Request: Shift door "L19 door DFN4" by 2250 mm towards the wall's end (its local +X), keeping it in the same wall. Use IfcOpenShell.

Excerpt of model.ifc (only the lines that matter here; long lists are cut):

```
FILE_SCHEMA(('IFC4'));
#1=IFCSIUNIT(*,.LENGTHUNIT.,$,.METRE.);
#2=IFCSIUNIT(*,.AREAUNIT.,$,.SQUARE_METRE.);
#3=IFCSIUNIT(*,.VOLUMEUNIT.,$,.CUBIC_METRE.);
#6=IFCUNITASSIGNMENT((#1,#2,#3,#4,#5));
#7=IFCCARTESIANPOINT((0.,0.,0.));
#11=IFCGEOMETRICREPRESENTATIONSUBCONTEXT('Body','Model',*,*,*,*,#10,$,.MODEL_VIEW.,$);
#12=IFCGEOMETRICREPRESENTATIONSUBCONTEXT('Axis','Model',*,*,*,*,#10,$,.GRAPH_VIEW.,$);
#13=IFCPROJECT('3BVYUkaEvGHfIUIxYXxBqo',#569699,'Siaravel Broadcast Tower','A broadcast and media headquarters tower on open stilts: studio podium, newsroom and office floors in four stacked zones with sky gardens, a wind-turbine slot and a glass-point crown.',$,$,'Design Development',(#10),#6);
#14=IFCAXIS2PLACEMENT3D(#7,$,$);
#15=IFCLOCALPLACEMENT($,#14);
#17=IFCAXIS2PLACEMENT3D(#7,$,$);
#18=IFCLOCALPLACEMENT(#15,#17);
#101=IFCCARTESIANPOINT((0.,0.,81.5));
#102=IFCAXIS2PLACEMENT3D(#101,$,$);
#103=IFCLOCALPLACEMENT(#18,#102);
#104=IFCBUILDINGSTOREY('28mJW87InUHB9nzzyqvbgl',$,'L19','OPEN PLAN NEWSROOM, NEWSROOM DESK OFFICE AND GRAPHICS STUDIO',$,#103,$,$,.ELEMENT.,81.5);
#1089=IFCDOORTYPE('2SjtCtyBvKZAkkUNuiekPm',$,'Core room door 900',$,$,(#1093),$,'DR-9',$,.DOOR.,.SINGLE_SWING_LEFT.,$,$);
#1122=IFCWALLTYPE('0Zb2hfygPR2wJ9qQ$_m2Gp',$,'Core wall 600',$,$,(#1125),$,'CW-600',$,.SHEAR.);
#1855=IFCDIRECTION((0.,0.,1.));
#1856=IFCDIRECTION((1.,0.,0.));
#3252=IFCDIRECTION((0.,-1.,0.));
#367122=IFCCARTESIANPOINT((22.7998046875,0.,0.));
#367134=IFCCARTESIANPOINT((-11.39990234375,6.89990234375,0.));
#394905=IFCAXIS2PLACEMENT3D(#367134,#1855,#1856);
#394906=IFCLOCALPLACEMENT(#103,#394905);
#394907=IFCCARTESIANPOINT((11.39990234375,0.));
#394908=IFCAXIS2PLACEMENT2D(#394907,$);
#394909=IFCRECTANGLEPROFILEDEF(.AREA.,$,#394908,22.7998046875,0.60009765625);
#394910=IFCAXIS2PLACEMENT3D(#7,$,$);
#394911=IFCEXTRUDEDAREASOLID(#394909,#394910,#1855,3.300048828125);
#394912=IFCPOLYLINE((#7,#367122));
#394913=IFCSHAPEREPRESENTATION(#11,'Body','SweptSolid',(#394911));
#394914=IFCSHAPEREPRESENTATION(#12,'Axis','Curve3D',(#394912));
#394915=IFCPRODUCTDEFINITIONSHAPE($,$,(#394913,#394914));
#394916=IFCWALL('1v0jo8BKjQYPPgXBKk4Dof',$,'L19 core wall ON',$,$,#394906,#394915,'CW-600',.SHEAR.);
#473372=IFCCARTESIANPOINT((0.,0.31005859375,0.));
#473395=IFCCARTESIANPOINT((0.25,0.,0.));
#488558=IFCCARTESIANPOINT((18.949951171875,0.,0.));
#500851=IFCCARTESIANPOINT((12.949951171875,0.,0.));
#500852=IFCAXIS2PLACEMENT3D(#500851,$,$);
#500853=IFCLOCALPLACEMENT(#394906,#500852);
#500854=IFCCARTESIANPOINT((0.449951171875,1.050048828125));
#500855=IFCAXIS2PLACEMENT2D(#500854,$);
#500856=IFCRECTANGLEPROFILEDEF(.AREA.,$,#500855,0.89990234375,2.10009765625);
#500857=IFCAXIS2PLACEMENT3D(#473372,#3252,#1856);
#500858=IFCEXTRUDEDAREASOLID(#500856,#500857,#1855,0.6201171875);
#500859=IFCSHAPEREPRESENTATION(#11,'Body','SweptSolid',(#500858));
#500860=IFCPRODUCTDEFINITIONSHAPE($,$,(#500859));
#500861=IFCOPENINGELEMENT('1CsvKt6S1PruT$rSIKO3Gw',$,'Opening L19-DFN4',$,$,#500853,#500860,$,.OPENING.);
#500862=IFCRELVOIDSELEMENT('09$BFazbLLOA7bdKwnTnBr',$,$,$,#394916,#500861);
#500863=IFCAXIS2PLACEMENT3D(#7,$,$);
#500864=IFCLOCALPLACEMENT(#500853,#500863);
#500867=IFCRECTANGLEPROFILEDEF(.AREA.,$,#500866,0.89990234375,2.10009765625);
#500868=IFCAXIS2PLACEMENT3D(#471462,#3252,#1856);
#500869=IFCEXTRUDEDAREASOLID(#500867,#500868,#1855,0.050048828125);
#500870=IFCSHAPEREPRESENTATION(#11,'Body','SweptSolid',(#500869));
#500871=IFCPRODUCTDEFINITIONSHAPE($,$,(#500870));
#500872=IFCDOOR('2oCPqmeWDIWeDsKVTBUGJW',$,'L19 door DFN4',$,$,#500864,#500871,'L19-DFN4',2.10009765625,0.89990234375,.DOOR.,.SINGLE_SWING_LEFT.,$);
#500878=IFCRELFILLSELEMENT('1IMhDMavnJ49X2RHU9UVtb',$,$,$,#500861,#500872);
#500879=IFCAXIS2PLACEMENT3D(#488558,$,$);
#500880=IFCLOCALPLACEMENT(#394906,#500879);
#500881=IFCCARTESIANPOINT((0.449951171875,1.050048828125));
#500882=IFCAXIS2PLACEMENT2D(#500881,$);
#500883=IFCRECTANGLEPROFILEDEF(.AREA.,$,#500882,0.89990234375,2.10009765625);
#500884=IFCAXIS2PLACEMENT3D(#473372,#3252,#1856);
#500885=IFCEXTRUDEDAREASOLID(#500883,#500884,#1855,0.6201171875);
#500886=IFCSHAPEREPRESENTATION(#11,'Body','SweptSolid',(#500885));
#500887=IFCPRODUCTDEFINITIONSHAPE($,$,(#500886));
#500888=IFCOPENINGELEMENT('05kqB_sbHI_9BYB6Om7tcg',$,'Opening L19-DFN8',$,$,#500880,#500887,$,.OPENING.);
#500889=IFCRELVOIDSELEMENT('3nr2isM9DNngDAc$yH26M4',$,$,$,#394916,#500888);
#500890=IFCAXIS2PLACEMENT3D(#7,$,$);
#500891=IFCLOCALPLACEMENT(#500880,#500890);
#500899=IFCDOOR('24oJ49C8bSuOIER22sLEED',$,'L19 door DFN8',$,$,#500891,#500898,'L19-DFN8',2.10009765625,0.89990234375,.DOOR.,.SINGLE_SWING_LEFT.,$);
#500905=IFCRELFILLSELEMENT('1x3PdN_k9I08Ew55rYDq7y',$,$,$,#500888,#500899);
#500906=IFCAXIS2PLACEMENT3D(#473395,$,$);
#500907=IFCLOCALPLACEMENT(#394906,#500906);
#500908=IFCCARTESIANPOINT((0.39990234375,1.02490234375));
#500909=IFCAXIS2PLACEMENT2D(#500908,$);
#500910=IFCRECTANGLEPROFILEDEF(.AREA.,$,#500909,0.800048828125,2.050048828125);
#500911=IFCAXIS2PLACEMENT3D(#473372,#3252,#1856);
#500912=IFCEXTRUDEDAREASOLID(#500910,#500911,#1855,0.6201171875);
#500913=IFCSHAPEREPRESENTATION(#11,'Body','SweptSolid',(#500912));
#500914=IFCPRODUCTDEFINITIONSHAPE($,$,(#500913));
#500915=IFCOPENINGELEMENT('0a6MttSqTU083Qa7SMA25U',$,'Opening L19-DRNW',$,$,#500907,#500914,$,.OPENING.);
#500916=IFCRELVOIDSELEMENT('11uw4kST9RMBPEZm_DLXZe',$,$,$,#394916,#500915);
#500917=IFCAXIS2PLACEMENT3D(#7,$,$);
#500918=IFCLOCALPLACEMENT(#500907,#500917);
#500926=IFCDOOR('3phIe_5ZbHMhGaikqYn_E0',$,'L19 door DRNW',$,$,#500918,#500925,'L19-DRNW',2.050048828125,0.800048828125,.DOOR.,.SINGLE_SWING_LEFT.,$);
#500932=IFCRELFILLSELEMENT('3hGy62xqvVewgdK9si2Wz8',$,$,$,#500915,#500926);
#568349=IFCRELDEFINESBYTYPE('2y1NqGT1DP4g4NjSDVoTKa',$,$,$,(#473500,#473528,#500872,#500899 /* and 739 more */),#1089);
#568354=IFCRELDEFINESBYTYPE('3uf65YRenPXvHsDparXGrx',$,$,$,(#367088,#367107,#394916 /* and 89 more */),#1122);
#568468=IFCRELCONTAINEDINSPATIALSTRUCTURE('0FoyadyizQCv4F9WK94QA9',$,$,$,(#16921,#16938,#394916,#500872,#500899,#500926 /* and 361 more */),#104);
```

```python
import ifcopenshell
import ifcopenshell.api.geometry
import ifcopenshell.util.placement
import ifcopenshell.util.unit

model = ifcopenshell.open("model.ifc")
unit_scale = ifcopenshell.util.unit.calculate_unit_scale(model)

door = model.by_guid("2oCPqmeWDIWeDsKVTBUGJW")
opening = door.FillsVoids[0].RelatingOpeningElement
wall = opening.VoidsElements[0].RelatingBuildingElement

wall_matrix = ifcopenshell.util.placement.get_local_placement(wall.ObjectPlacement)
shift = wall_matrix[:3, 0] * 2.25 / unit_scale
before = ifcopenshell.util.placement.get_local_placement(door.ObjectPlacement)[:3, 3].copy()

# The door is placed relative to its opening, so it follows when the opening moves.
matrix = ifcopenshell.util.placement.get_local_placement(opening.ObjectPlacement)
matrix[:3, 3] += shift
ifcopenshell.api.geometry.edit_object_placement(
    model, product=opening, matrix=matrix, is_si=False, should_transform_children=True
)

after = ifcopenshell.util.placement.get_local_placement(door.ObjectPlacement)[:3, 3]
print("door moved by", (after - before).round(3) + 0.0)

model.write("model_v2.ifc")
```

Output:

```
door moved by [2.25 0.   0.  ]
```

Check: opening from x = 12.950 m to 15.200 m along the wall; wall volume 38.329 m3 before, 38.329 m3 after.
